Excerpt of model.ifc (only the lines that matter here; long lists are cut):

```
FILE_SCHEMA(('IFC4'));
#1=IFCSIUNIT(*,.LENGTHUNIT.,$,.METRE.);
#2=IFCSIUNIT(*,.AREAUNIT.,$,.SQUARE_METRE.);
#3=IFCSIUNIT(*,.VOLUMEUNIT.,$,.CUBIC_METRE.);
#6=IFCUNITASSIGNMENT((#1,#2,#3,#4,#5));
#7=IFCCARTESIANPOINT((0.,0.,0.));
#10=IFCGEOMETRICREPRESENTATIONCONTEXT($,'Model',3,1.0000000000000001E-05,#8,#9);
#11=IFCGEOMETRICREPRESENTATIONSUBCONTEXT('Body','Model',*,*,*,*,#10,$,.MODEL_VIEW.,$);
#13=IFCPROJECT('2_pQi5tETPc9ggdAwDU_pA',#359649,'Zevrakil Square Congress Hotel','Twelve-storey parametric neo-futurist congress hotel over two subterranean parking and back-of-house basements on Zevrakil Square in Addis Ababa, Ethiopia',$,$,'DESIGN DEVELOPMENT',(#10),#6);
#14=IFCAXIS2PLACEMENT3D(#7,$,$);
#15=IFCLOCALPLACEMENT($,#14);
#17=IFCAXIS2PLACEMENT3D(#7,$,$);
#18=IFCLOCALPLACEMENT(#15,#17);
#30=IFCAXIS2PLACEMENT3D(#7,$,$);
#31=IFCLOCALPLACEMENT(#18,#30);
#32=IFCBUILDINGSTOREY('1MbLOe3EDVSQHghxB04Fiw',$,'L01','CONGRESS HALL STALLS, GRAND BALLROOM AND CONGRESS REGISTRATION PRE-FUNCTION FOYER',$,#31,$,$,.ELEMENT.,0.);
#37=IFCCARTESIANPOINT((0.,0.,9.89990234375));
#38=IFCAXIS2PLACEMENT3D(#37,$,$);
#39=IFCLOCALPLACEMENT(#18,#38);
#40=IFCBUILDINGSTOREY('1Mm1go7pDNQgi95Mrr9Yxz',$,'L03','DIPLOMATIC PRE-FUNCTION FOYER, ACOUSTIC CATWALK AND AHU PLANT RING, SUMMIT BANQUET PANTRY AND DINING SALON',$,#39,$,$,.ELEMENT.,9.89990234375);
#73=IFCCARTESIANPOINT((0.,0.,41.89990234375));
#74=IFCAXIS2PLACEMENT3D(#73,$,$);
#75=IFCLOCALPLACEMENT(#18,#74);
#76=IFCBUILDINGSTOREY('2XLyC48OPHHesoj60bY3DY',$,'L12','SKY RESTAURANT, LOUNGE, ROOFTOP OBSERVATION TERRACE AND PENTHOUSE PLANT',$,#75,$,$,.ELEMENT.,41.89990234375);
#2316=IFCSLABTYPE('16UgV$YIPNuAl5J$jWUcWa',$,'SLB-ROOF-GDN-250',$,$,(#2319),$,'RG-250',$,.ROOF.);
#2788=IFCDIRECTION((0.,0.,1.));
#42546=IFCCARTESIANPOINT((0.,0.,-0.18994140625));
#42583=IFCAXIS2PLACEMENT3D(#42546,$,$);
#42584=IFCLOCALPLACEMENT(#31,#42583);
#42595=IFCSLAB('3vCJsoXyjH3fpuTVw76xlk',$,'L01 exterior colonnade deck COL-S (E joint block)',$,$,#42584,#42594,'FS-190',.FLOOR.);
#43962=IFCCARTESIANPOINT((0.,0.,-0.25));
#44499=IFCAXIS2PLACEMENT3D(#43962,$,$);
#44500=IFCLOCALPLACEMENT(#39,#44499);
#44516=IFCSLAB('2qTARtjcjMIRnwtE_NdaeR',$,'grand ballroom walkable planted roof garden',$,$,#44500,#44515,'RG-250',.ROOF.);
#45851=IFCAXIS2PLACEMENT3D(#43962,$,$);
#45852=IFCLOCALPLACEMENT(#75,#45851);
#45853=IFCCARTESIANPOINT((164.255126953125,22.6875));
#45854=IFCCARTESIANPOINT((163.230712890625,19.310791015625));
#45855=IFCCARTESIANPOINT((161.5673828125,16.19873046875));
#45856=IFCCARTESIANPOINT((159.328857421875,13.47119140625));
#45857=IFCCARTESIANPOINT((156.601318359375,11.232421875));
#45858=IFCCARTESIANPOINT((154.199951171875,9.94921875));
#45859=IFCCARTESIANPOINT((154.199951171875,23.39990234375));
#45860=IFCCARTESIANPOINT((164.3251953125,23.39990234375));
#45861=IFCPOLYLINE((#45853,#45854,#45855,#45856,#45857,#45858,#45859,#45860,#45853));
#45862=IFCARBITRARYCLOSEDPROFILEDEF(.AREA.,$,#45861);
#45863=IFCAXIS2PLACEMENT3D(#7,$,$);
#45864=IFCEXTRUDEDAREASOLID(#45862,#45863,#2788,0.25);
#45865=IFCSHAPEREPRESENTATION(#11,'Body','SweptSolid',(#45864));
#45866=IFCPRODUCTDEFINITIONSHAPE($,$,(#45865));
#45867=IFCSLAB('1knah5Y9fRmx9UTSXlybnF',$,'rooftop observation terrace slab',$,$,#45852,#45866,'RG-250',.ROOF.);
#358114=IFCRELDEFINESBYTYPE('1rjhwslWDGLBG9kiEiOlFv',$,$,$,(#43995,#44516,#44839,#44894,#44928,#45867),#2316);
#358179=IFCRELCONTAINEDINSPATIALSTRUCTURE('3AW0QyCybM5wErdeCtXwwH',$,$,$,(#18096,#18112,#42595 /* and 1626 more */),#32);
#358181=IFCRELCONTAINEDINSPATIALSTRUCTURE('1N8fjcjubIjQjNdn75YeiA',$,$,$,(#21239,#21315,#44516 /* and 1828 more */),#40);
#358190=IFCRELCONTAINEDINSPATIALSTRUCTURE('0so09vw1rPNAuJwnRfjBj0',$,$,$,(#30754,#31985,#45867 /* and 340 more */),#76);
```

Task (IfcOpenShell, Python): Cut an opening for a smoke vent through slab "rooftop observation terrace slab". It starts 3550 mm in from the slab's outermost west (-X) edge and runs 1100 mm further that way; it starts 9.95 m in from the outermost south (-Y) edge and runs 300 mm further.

```python
import numpy as np
import ifcopenshell
import ifcopenshell.api.feature
import ifcopenshell.api.geometry
import ifcopenshell.api.root
import ifcopenshell.geom
import ifcopenshell.util.placement
import ifcopenshell.util.representation
import ifcopenshell.util.shape
import ifcopenshell.util.unit

model = ifcopenshell.open("model.ifc")
unit_scale = ifcopenshell.util.unit.calculate_unit_scale(model)
settings = ifcopenshell.geom.settings()


def volume(element):
    """Net volume in cubic metres, openings subtracted."""
    shape = ifcopenshell.geom.create_shape(settings, element)
    return ifcopenshell.util.shape.get_volume(shape.geometry)


slab = model.by_guid("1knah5Y9fRmx9UTSXlybnF")
before = volume(slab)

# Extent in the slab's own axes, in metres. The edges named are its -X and -Y sides.
slab_shape = ifcopenshell.geom.create_shape(settings, slab)
vertices = ifcopenshell.util.shape.get_vertices(slab_shape.geometry)
x_min, y_min, bottom = vertices.min(axis=0)
top = vertices[:, 2].max()

opening = ifcopenshell.api.root.create_entity(model, ifc_class="IfcOpeningElement", name="Smoke vent opening", predefined_type="OPENING")
context = ifcopenshell.util.representation.get_context(model, "Model", "Body", "MODEL_VIEW")
width, depth = 1.1, 0.3
outline = [(0.0, 0.0), (width, 0.0), (width, depth), (0.0, depth), (0.0, 0.0)]
# Overshoot both faces by 50 mm so the cut is clean.
shape = ifcopenshell.api.geometry.add_slab_representation(
    model, context=context, depth=top - bottom + 0.1, polyline=outline
)
ifcopenshell.api.geometry.assign_representation(model, product=opening, representation=shape)

matrix = ifcopenshell.util.placement.get_local_placement(slab.ObjectPlacement)
matrix[:, 3] = matrix @ np.append(np.array([x_min + 3.55, y_min + 9.95, bottom - 0.05]) / unit_scale, 1.0)
ifcopenshell.api.geometry.edit_object_placement(model, product=opening, matrix=matrix, is_si=False)
ifcopenshell.api.feature.add_feature(model, feature=opening, element=slab)

after = volume(slab)

print(f"slab volume {before:.3f} -> {after:.3f} m3")

model.write("model_v2.ifc")
```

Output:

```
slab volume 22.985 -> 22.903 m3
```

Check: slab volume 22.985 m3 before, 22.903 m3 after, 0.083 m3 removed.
